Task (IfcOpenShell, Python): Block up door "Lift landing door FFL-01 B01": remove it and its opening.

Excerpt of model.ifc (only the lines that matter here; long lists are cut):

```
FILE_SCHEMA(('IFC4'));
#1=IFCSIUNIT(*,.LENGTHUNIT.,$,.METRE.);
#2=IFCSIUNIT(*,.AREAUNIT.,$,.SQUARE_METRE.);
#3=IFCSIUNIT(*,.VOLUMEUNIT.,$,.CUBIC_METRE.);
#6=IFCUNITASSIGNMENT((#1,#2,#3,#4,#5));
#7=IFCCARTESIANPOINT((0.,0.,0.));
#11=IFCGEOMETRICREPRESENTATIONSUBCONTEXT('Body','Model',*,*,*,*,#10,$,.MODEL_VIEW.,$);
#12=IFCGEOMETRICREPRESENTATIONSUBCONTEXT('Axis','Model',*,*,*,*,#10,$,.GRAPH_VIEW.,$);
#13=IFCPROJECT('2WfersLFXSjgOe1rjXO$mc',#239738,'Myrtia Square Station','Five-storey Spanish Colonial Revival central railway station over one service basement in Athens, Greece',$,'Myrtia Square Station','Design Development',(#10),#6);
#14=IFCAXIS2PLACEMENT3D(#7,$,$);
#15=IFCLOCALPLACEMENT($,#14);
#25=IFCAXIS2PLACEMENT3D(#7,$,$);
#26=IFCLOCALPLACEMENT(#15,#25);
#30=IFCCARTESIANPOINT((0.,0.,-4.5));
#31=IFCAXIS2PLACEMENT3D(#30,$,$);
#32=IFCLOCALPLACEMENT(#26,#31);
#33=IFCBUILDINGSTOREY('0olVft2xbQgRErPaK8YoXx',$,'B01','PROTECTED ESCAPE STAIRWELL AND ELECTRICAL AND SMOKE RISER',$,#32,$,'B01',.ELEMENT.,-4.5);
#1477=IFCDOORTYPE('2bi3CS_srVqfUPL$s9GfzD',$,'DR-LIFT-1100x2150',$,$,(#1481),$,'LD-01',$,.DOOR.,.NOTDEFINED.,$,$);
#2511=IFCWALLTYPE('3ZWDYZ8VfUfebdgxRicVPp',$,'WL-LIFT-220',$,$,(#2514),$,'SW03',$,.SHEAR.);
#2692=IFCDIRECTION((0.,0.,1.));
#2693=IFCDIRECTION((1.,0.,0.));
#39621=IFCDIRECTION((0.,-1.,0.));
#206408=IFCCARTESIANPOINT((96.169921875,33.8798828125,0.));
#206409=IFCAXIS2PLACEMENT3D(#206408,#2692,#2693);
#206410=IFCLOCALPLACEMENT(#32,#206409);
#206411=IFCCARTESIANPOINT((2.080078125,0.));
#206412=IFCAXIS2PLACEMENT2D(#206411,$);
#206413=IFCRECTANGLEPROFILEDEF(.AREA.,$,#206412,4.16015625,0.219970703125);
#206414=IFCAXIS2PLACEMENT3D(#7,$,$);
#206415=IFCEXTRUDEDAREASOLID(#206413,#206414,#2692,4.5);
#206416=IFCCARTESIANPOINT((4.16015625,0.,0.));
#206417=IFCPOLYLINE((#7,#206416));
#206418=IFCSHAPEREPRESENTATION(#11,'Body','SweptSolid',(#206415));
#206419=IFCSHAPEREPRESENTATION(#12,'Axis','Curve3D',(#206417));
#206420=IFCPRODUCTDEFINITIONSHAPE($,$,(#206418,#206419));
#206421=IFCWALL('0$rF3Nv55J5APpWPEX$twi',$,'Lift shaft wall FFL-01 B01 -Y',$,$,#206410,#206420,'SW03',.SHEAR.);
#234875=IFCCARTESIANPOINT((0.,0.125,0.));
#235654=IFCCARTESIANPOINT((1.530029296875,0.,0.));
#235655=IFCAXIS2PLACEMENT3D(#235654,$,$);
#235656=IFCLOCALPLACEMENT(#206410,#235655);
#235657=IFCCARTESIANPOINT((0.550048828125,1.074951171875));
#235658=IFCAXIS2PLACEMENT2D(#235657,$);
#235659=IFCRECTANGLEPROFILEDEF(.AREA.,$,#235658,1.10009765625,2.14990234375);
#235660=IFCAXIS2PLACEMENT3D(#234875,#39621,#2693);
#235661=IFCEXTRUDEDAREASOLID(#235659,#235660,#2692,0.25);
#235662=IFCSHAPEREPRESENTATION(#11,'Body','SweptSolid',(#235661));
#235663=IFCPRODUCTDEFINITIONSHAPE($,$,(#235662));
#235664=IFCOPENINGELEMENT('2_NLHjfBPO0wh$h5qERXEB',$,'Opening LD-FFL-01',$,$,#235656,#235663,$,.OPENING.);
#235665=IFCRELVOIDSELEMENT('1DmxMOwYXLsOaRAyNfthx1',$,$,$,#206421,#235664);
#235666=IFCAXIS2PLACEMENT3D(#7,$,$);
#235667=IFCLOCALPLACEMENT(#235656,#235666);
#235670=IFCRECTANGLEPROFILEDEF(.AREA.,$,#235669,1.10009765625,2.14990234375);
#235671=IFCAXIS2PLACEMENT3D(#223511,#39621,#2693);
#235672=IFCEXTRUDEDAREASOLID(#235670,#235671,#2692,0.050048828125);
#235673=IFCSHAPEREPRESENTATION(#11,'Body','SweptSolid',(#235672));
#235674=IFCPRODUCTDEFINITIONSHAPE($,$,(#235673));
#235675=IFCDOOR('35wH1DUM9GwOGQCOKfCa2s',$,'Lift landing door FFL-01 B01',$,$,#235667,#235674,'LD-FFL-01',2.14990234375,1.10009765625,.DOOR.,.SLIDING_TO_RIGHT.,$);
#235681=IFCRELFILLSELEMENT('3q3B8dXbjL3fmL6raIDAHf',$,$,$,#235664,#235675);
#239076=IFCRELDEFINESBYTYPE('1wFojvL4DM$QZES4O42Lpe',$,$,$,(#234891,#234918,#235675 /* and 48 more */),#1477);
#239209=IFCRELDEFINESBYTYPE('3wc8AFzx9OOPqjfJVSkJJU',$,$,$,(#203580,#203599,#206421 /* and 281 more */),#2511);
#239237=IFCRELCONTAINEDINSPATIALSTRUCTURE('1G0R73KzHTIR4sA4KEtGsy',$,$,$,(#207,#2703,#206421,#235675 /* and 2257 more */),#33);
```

```python
import ifcopenshell
import ifcopenshell.api.feature
import ifcopenshell.api.root
import ifcopenshell.geom
import ifcopenshell.util.shape

model = ifcopenshell.open("model.ifc")
settings = ifcopenshell.geom.settings()


def volume(element):
    """Net volume in cubic metres, openings subtracted."""
    shape = ifcopenshell.geom.create_shape(settings, element)
    return ifcopenshell.util.shape.get_volume(shape.geometry)


door = model.by_guid("35wH1DUM9GwOGQCOKfCa2s")
opening = door.FillsVoids[0].RelatingOpeningElement
wall = opening.VoidsElements[0].RelatingBuildingElement
before = volume(wall)

ifcopenshell.api.root.remove_product(model, product=door)
ifcopenshell.api.feature.remove_feature(model, feature=opening)

after = volume(wall)

print(f"wall volume {before:.3f} -> {after:.3f} m3")

model.write("model_rev.ifc")
```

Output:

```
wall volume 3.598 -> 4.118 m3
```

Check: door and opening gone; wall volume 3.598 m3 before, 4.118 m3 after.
